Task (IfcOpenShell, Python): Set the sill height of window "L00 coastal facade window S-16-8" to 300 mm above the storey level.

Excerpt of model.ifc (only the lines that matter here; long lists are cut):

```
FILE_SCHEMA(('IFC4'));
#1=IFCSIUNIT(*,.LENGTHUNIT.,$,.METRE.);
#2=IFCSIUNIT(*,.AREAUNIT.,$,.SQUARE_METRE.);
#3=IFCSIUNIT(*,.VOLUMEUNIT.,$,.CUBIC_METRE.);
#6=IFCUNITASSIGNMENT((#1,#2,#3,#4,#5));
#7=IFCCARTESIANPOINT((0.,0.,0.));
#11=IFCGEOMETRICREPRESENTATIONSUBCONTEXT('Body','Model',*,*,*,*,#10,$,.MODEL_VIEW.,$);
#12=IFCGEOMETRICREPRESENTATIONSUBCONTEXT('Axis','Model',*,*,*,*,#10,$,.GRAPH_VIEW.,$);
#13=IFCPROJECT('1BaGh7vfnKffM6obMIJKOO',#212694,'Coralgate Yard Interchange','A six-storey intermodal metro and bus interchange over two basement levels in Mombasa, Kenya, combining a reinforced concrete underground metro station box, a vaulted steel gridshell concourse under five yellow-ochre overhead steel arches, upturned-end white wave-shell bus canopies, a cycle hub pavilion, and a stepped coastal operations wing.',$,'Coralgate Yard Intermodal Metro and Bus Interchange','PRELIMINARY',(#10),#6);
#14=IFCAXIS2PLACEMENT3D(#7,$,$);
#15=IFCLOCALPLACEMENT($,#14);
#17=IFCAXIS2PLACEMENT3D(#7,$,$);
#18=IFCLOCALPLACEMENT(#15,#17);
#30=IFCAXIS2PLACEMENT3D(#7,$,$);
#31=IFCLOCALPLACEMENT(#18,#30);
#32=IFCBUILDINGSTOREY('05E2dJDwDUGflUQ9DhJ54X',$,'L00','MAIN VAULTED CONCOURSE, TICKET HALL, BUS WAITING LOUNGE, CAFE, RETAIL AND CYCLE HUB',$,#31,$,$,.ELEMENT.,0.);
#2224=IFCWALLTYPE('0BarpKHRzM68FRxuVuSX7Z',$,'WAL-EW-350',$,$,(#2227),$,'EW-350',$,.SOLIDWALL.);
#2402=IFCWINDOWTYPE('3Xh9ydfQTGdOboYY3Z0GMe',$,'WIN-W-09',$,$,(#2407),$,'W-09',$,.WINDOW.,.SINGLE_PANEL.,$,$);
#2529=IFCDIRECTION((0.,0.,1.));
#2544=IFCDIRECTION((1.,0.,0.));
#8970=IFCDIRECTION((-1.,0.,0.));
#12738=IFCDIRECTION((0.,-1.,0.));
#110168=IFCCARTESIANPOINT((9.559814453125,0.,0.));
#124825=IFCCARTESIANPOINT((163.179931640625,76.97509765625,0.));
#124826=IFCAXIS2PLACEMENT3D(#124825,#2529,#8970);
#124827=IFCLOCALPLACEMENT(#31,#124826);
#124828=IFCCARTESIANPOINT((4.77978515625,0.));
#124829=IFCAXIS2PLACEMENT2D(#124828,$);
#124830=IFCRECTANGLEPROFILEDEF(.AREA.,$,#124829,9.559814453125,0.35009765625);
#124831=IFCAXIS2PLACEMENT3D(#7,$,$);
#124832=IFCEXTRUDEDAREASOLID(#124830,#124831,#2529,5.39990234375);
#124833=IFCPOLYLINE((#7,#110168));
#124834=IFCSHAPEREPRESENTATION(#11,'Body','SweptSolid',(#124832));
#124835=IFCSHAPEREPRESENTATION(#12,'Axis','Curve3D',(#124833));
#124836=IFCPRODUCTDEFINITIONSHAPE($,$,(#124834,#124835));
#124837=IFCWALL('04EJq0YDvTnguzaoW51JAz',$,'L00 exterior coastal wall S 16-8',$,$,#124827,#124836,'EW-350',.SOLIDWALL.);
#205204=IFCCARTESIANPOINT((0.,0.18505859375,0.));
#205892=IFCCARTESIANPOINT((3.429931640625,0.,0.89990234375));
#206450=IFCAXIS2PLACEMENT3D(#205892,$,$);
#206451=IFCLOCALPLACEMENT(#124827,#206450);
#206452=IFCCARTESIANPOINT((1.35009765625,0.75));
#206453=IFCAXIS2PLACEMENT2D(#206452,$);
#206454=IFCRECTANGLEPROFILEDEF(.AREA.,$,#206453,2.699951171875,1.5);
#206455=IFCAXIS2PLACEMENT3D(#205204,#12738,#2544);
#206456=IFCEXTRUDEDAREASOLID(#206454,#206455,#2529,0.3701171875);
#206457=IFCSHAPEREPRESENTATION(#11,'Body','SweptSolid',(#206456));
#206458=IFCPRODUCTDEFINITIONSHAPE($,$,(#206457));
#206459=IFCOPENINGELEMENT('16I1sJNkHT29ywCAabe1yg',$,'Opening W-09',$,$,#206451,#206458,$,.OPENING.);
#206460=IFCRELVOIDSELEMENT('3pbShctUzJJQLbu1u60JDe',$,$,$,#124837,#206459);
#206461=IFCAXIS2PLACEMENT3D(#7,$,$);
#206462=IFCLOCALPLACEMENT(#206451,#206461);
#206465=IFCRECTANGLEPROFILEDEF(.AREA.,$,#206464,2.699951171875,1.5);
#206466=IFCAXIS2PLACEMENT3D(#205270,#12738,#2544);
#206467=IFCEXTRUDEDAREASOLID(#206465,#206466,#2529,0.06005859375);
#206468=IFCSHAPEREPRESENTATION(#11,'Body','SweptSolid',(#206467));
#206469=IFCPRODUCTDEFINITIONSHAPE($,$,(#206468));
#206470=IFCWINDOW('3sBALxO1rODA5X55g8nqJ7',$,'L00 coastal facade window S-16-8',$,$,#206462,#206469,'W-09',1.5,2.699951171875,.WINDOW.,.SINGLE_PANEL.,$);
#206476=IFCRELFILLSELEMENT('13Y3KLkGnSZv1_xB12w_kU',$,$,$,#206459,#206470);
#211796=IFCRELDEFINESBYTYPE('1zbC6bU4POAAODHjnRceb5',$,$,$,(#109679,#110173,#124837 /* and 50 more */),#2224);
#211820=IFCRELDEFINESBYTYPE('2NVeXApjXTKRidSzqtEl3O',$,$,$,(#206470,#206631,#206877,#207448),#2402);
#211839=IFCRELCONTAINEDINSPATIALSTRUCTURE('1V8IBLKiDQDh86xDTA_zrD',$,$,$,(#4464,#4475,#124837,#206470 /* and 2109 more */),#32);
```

```python
import numpy as np
import ifcopenshell
import ifcopenshell.api.geometry
import ifcopenshell.geom
import ifcopenshell.util.element
import ifcopenshell.util.placement
import ifcopenshell.util.shape
import ifcopenshell.util.unit

model = ifcopenshell.open("model.ifc")
unit_scale = ifcopenshell.util.unit.calculate_unit_scale(model)

window = model.by_id(206470)
opening = window.FillsVoids[0].RelatingOpeningElement
storey = ifcopenshell.util.element.get_container(window, ifc_class="IfcBuildingStorey")
level = ifcopenshell.util.placement.get_local_placement(storey.ObjectPlacement)[2, 3]

# The opening's origin need not be at the sill, so measure its lowest point.
shape = ifcopenshell.geom.create_shape(ifcopenshell.geom.settings(), opening)
bottom = ifcopenshell.util.shape.get_shape_bottom_elevation(shape, shape.geometry) / unit_scale
dz = level + 0.3 / unit_scale - bottom

shift = np.array([0.0, 0.0, dz])
# The window is placed relative to its opening, so it follows when the opening moves.
matrix = ifcopenshell.util.placement.get_local_placement(opening.ObjectPlacement)
matrix[:3, 3] += shift
ifcopenshell.api.geometry.edit_object_placement(
    model, product=opening, matrix=matrix, is_si=False, should_transform_children=True
)

print(f"moved by {dz * unit_scale:+.3f} m")

model.write("model_rev.ifc")
```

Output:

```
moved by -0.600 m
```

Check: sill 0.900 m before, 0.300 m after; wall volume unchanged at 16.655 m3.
